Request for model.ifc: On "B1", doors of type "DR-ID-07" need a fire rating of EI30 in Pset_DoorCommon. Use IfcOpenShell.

First a look at what the model holds.

```python
import ifcopenshell
import ifcopenshell.util.element

model = ifcopenshell.open("model.ifc")
print(model.schema)
storey = next(s for s in model.by_type("IfcBuildingStorey") if s.Name == "B1")
doors = [e for e in ifcopenshell.util.element.get_decomposition(storey) if e.is_a("IfcDoor")]
seen = {}
for e in doors:
    element_type = ifcopenshell.util.element.get_type(e)
    key = (element_type.Name if element_type != e and element_type else None, ifcopenshell.util.element.get_pset(e, "Pset_DoorCommon", "FireRating"))
    seen[key] = seen.get(key, 0) + 1
for (name, value), count in sorted(seen.items(), key=str):
    print(count, "x", name, "|", value)
```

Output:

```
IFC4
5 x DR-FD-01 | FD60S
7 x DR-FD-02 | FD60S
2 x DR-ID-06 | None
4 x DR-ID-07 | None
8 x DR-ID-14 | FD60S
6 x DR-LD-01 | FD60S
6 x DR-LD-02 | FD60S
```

```python
import ifcopenshell
import ifcopenshell.api.pset
import ifcopenshell.util.element

model = ifcopenshell.open("model.ifc")

storey = next(s for s in model.by_type("IfcBuildingStorey") if s.Name == "B1")
doors = [e for e in ifcopenshell.util.element.get_decomposition(storey) if e.is_a("IfcDoor")]

count = 0
for e in doors:
    element_type = ifcopenshell.util.element.get_type(e)
    if element_type in (None, e) or element_type.Name != "DR-ID-07":
        continue
    # add_pset returns the element's existing set when there is one.
    pset = ifcopenshell.api.pset.add_pset(model, product=e, name="Pset_DoorCommon")
    ifcopenshell.api.pset.edit_pset(model, pset=pset, properties={"FireRating": "EI30"})
    count += 1

print(count, "doors updated")

model.write("model_edited.ifc")
```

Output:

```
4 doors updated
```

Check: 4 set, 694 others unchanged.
